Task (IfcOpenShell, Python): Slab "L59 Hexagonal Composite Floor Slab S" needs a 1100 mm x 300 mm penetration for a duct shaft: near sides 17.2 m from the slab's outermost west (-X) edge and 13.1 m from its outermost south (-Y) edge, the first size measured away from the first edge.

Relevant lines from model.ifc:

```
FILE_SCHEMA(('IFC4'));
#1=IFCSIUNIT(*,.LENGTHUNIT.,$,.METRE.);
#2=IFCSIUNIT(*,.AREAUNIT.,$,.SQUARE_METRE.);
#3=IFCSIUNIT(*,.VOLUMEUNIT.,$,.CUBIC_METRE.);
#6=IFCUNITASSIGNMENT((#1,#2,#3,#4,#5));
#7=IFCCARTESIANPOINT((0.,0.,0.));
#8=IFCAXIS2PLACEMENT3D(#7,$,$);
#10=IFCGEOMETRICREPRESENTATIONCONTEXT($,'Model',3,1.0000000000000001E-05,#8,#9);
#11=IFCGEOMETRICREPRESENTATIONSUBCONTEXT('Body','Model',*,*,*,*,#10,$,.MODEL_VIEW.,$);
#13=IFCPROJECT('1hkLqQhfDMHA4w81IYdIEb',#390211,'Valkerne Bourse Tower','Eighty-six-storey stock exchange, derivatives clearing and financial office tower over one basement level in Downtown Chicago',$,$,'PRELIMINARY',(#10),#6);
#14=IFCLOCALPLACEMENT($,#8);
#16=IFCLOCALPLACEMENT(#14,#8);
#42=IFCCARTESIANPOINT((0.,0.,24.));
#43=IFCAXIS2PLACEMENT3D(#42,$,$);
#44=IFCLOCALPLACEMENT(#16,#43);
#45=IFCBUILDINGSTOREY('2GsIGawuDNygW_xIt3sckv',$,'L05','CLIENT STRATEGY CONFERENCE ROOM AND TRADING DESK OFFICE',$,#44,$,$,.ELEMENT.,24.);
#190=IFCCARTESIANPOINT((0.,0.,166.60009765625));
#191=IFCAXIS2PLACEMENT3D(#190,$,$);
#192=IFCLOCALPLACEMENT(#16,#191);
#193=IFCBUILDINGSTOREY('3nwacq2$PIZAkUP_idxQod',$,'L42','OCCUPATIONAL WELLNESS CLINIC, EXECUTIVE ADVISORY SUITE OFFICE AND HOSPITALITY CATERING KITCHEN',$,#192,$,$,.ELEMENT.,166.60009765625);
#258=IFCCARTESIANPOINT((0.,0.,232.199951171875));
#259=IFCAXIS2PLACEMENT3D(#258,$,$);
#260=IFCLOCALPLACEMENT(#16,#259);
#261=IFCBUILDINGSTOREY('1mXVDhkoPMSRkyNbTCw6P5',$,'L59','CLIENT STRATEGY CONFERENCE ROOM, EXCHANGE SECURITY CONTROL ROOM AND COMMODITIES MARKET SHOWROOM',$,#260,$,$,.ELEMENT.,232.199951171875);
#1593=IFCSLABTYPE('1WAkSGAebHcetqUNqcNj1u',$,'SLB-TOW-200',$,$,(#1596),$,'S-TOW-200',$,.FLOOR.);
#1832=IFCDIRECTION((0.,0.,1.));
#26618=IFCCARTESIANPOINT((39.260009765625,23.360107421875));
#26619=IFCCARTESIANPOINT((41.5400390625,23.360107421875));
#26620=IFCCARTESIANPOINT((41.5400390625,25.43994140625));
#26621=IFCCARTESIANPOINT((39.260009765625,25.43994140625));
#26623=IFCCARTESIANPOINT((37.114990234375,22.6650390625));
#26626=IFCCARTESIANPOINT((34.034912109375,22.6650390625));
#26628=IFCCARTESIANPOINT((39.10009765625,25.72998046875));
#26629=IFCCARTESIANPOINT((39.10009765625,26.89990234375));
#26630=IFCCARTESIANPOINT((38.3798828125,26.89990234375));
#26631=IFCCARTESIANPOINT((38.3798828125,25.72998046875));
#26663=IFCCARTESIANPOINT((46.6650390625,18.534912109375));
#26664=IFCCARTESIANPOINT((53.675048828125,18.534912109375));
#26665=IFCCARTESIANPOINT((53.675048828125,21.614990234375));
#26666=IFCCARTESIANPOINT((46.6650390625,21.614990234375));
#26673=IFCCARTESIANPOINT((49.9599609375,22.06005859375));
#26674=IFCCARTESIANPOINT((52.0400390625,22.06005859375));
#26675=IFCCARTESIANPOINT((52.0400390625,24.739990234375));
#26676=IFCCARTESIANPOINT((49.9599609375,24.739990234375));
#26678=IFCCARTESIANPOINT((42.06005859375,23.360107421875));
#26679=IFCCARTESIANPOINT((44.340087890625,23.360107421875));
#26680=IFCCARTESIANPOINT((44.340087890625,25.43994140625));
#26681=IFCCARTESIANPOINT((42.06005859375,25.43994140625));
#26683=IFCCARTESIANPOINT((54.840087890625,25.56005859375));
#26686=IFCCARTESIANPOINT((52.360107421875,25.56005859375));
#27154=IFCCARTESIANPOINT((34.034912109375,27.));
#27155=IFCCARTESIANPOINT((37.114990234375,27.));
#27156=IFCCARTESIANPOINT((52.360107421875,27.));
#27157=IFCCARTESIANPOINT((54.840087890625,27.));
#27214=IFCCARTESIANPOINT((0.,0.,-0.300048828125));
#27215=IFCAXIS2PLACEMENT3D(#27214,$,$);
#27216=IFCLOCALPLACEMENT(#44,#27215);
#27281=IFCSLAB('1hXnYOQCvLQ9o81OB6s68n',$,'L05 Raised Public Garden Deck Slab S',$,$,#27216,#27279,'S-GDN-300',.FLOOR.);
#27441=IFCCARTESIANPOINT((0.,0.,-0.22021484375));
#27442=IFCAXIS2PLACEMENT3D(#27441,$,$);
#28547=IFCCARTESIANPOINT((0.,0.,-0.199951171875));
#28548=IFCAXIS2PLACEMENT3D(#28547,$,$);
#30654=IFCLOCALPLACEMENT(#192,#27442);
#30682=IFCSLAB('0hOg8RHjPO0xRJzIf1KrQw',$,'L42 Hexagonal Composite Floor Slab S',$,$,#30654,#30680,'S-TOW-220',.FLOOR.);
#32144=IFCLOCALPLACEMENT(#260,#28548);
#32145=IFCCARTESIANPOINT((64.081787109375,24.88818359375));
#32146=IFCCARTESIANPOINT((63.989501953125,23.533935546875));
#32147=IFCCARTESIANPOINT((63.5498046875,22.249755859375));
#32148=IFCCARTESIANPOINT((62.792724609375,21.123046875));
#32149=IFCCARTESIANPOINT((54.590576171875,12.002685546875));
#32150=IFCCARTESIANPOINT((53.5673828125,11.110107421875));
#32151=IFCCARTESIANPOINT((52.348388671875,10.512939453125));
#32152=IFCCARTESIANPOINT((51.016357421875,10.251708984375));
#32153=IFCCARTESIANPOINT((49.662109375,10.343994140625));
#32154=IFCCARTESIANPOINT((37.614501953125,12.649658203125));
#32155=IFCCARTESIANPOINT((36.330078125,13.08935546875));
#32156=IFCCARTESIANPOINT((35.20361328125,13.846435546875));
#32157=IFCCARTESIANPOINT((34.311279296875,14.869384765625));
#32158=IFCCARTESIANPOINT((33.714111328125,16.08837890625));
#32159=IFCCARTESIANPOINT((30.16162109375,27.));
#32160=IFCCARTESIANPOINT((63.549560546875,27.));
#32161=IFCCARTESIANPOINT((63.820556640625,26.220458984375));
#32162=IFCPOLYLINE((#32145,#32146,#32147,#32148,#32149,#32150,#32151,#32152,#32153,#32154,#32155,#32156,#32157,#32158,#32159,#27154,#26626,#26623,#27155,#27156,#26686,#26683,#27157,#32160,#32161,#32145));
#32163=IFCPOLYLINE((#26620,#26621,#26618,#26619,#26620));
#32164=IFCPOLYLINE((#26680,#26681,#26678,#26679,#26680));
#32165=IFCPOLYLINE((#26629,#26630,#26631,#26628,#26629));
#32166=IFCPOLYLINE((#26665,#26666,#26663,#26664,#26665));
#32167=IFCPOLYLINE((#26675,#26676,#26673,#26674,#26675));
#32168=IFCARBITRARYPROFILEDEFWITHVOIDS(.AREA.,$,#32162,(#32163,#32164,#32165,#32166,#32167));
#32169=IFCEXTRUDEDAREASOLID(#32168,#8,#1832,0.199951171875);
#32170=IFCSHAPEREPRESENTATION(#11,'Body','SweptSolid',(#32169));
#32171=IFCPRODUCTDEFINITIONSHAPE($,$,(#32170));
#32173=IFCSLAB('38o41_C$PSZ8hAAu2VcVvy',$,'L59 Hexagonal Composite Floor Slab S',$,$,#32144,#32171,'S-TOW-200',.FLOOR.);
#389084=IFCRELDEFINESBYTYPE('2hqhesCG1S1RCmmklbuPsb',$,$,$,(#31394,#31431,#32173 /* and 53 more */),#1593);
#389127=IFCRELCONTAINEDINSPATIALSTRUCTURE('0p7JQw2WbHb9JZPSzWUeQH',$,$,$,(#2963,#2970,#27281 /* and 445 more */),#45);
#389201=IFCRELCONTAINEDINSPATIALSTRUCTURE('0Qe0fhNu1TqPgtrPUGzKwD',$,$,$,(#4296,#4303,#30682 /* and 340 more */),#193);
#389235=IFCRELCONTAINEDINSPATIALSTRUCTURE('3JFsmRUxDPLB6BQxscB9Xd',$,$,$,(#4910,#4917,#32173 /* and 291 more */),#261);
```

```python
import numpy as np
import ifcopenshell
import ifcopenshell.api.feature
import ifcopenshell.api.geometry
import ifcopenshell.api.root
import ifcopenshell.geom
import ifcopenshell.util.placement
import ifcopenshell.util.representation
import ifcopenshell.util.shape
import ifcopenshell.util.unit

model = ifcopenshell.open("model.ifc")
unit_scale = ifcopenshell.util.unit.calculate_unit_scale(model)
settings = ifcopenshell.geom.settings()


def volume(element):
    """Net volume in cubic metres, openings subtracted."""
    shape = ifcopenshell.geom.create_shape(settings, element)
    return ifcopenshell.util.shape.get_volume(shape.geometry)


slab = model.by_guid("38o41_C$PSZ8hAAu2VcVvy")
before = volume(slab)

# Extent in the slab's own axes, in metres. The edges named are its -X and -Y sides.
slab_shape = ifcopenshell.geom.create_shape(settings, slab)
vertices = ifcopenshell.util.shape.get_vertices(slab_shape.geometry)
x_min, y_min, bottom = vertices.min(axis=0)
top = vertices[:, 2].max()

opening = ifcopenshell.api.root.create_entity(model, ifc_class="IfcOpeningElement", name="Duct shaft opening", predefined_type="OPENING")
context = ifcopenshell.util.representation.get_context(model, "Model", "Body", "MODEL_VIEW")
width, depth = 1.1, 0.3
outline = [(0.0, 0.0), (width, 0.0), (width, depth), (0.0, depth), (0.0, 0.0)]
# Overshoot both faces by 50 mm so the cut is clean.
shape = ifcopenshell.api.geometry.add_slab_representation(
    model, context=context, depth=top - bottom + 0.1, polyline=outline
)
ifcopenshell.api.geometry.assign_representation(model, product=opening, representation=shape)

matrix = ifcopenshell.util.placement.get_local_placement(slab.ObjectPlacement)
matrix[:, 3] = matrix @ np.append(np.array([x_min + 17.2, y_min + 13.1, bottom - 0.05]) / unit_scale, 1.0)
ifcopenshell.api.geometry.edit_object_placement(model, product=opening, matrix=matrix, is_si=False)
ifcopenshell.api.feature.add_feature(model, feature=opening, element=slab)

after = volume(slab)

print(f"slab volume {before:.3f} -> {after:.3f} m3")

model.write("model-out.ifc")
```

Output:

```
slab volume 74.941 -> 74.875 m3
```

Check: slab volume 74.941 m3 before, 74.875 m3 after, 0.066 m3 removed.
